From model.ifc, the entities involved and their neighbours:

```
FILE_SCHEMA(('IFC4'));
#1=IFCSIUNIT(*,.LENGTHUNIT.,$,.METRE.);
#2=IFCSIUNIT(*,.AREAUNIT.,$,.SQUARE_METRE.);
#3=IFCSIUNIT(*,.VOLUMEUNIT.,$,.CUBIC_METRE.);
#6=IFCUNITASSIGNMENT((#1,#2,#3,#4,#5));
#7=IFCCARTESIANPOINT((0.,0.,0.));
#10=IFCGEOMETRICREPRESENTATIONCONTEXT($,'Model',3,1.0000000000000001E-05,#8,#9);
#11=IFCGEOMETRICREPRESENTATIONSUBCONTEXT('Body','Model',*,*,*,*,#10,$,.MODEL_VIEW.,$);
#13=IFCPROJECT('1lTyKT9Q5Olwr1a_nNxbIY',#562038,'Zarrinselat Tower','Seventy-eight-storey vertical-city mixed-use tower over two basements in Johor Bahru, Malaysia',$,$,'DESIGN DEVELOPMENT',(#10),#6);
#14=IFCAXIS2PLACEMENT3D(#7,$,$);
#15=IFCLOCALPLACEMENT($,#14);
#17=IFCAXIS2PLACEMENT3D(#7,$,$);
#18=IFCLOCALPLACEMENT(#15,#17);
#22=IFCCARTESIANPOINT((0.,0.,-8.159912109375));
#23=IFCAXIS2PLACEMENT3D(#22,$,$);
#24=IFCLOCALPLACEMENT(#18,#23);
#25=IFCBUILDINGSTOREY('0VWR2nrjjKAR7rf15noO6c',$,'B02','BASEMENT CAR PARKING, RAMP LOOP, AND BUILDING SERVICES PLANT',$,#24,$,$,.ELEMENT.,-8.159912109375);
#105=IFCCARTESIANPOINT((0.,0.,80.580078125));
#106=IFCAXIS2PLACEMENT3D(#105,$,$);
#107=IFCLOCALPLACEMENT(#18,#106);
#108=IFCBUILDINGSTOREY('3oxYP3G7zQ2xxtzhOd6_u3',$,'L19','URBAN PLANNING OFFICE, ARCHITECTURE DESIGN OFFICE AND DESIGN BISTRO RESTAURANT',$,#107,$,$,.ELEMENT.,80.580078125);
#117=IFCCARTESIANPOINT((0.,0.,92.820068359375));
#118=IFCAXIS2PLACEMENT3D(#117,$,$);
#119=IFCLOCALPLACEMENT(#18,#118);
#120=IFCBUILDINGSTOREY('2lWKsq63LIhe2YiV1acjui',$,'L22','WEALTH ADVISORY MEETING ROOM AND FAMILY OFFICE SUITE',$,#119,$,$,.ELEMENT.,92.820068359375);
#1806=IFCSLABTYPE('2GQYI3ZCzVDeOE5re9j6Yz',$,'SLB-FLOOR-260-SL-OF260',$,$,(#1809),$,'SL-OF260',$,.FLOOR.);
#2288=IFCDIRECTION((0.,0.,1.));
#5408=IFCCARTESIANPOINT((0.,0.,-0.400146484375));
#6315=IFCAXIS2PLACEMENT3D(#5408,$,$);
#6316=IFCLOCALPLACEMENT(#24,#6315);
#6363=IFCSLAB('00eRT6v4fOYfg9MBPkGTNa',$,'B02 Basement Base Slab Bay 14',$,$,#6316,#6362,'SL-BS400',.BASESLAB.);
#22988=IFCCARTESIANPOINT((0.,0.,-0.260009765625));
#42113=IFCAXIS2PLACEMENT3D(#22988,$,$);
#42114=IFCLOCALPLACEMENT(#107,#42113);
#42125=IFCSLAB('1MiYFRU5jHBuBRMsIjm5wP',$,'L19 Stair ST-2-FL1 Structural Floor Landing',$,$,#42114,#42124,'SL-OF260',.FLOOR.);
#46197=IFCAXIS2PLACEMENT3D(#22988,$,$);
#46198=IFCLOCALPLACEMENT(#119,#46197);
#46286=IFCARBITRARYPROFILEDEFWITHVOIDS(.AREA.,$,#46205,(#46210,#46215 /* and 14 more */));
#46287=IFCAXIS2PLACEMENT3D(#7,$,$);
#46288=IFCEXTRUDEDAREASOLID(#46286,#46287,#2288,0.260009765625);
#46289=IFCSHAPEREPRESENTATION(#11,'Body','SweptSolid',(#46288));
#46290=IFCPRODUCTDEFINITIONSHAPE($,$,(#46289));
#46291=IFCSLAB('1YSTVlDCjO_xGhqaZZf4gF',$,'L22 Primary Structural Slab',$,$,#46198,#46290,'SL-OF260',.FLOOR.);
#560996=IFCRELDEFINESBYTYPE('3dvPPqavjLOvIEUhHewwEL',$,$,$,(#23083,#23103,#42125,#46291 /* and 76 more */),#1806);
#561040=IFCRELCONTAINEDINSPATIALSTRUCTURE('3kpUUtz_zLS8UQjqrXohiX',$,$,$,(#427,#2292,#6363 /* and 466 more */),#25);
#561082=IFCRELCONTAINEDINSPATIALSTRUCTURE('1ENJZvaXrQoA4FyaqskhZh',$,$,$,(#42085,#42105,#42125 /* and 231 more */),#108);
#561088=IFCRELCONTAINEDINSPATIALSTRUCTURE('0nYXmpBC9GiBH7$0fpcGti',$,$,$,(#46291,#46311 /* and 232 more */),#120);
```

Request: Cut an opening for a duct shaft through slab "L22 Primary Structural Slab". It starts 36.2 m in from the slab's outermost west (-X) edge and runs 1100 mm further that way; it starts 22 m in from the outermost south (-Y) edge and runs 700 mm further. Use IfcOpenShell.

```python
import numpy as np
import ifcopenshell
import ifcopenshell.api.feature
import ifcopenshell.api.geometry
import ifcopenshell.api.root
import ifcopenshell.geom
import ifcopenshell.util.placement
import ifcopenshell.util.representation
import ifcopenshell.util.shape
import ifcopenshell.util.unit

model = ifcopenshell.open("model.ifc")
unit_scale = ifcopenshell.util.unit.calculate_unit_scale(model)
settings = ifcopenshell.geom.settings()


def volume(element):
    """Net volume in cubic metres, openings subtracted."""
    shape = ifcopenshell.geom.create_shape(settings, element)
    return ifcopenshell.util.shape.get_volume(shape.geometry)


slab = model.by_guid("1YSTVlDCjO_xGhqaZZf4gF")
before = volume(slab)

# Extent in the slab's own axes, in metres. The edges named are its -X and -Y sides.
slab_shape = ifcopenshell.geom.create_shape(settings, slab)
vertices = ifcopenshell.util.shape.get_vertices(slab_shape.geometry)
x_min, y_min, bottom = vertices.min(axis=0)
top = vertices[:, 2].max()

opening = ifcopenshell.api.root.create_entity(model, ifc_class="IfcOpeningElement", name="Duct shaft opening", predefined_type="OPENING")
context = ifcopenshell.util.representation.get_context(model, "Model", "Body", "MODEL_VIEW")
width, depth = 1.1, 0.7
outline = [(0.0, 0.0), (width, 0.0), (width, depth), (0.0, depth), (0.0, 0.0)]
# Overshoot both faces by 50 mm so the cut is clean.
shape = ifcopenshell.api.geometry.add_slab_representation(
    model, context=context, depth=top - bottom + 0.1, polyline=outline
)
ifcopenshell.api.geometry.assign_representation(model, product=opening, representation=shape)

matrix = ifcopenshell.util.placement.get_local_placement(slab.ObjectPlacement)
matrix[:, 3] = matrix @ np.append(np.array([x_min + 36.2, y_min + 22, bottom - 0.05]) / unit_scale, 1.0)
ifcopenshell.api.geometry.edit_object_placement(model, product=opening, matrix=matrix, is_si=False)
ifcopenshell.api.feature.add_feature(model, feature=opening, element=slab)

after = volume(slab)

print(f"slab volume {before:.3f} -> {after:.3f} m3")

model.write("model_v2.ifc")
```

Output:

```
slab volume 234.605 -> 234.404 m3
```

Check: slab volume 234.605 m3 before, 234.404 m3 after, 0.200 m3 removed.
